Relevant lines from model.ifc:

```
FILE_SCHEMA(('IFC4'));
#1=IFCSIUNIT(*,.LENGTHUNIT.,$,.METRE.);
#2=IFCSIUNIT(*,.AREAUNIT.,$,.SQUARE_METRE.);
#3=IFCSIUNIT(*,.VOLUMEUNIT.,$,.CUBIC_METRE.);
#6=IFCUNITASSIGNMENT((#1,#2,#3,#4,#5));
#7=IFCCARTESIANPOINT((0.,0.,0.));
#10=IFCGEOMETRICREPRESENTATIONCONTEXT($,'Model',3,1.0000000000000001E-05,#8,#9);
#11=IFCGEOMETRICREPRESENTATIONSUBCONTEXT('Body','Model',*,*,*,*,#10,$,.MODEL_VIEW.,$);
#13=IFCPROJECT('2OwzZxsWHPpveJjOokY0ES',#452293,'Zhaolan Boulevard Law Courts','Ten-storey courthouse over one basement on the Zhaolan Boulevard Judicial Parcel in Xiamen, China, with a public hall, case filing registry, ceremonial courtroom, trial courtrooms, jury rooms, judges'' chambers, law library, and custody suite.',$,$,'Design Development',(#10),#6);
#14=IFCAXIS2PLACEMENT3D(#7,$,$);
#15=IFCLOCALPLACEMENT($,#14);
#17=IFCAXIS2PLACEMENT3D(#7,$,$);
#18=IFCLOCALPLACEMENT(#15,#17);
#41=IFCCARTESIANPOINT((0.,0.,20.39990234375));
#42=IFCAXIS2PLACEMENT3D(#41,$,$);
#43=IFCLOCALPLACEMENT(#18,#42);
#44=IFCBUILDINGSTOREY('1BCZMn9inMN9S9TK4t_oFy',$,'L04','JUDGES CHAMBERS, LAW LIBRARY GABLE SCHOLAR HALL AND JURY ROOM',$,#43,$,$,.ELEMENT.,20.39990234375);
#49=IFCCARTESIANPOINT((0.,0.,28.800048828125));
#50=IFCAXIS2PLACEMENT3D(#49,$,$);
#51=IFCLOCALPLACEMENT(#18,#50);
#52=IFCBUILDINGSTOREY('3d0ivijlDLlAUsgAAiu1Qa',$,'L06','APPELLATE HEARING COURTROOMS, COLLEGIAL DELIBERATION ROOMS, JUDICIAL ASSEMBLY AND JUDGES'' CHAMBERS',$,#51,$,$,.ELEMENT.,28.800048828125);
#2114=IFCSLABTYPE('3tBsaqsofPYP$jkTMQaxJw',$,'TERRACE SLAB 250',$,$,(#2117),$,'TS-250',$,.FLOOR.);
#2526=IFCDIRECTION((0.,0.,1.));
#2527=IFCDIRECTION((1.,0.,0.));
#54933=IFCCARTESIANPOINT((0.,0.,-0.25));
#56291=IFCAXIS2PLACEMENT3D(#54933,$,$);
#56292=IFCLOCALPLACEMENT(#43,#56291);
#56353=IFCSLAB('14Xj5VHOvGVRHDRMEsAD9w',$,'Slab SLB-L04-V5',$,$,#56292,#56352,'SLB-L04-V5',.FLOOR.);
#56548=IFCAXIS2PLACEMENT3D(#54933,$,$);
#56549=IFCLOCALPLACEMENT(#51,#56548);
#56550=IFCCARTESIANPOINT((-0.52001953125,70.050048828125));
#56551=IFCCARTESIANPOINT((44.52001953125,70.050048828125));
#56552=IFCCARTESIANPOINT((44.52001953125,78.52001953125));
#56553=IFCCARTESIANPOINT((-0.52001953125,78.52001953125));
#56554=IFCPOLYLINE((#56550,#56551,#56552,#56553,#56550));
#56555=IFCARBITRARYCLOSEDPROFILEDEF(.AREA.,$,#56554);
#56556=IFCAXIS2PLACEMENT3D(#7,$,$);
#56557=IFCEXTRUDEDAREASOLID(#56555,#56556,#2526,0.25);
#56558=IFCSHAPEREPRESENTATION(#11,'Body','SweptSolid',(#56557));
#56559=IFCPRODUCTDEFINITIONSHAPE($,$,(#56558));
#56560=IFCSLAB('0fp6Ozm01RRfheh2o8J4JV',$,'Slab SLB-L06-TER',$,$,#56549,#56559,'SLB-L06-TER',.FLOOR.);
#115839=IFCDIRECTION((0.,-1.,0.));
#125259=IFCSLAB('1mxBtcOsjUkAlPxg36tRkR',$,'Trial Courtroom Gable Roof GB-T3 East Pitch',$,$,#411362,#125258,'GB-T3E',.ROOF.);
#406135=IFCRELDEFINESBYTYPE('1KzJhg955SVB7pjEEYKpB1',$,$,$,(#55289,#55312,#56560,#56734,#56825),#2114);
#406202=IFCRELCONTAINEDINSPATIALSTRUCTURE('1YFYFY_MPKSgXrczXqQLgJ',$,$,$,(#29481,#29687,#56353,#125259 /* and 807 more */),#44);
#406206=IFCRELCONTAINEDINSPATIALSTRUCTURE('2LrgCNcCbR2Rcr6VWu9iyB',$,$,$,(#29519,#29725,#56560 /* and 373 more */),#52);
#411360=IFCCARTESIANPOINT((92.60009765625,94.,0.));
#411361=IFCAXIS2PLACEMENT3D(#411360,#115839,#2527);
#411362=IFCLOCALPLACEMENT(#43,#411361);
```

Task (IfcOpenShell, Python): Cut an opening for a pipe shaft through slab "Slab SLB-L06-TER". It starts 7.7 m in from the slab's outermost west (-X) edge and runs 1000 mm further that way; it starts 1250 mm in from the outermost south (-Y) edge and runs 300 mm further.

```python
import numpy as np
import ifcopenshell
import ifcopenshell.api.feature
import ifcopenshell.api.geometry
import ifcopenshell.api.root
import ifcopenshell.geom
import ifcopenshell.util.placement
import ifcopenshell.util.representation
import ifcopenshell.util.shape
import ifcopenshell.util.unit

model = ifcopenshell.open("model.ifc")
unit_scale = ifcopenshell.util.unit.calculate_unit_scale(model)
settings = ifcopenshell.geom.settings()


def volume(element):
    """Net volume in cubic metres, openings subtracted."""
    shape = ifcopenshell.geom.create_shape(settings, element)
    return ifcopenshell.util.shape.get_volume(shape.geometry)


slab = model.by_guid("0fp6Ozm01RRfheh2o8J4JV")
before = volume(slab)

# Extent in the slab's own axes, in metres. The edges named are its -X and -Y sides.
slab_shape = ifcopenshell.geom.create_shape(settings, slab)
vertices = ifcopenshell.util.shape.get_vertices(slab_shape.geometry)
x_min, y_min, bottom = vertices.min(axis=0)
top = vertices[:, 2].max()

opening = ifcopenshell.api.root.create_entity(model, ifc_class="IfcOpeningElement", name="Pipe shaft opening", predefined_type="OPENING")
context = ifcopenshell.util.representation.get_context(model, "Model", "Body", "MODEL_VIEW")
width, depth = 1, 0.3
outline = [(0.0, 0.0), (width, 0.0), (width, depth), (0.0, depth), (0.0, 0.0)]
# Overshoot both faces by 50 mm so the cut is clean.
shape = ifcopenshell.api.geometry.add_slab_representation(
    model, context=context, depth=top - bottom + 0.1, polyline=outline
)
ifcopenshell.api.geometry.assign_representation(model, product=opening, representation=shape)

matrix = ifcopenshell.util.placement.get_local_placement(slab.ObjectPlacement)
matrix[:, 3] = matrix @ np.append(np.array([x_min + 7.7, y_min + 1.25, bottom - 0.05]) / unit_scale, 1.0)
ifcopenshell.api.geometry.edit_object_placement(model, product=opening, matrix=matrix, is_si=False)
ifcopenshell.api.feature.add_feature(model, feature=opening, element=slab)

after = volume(slab)

print(f"slab volume {before:.3f} -> {after:.3f} m3")

model.write("model_v2.ifc")
```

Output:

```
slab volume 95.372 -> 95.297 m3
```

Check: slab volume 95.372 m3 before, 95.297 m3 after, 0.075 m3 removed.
